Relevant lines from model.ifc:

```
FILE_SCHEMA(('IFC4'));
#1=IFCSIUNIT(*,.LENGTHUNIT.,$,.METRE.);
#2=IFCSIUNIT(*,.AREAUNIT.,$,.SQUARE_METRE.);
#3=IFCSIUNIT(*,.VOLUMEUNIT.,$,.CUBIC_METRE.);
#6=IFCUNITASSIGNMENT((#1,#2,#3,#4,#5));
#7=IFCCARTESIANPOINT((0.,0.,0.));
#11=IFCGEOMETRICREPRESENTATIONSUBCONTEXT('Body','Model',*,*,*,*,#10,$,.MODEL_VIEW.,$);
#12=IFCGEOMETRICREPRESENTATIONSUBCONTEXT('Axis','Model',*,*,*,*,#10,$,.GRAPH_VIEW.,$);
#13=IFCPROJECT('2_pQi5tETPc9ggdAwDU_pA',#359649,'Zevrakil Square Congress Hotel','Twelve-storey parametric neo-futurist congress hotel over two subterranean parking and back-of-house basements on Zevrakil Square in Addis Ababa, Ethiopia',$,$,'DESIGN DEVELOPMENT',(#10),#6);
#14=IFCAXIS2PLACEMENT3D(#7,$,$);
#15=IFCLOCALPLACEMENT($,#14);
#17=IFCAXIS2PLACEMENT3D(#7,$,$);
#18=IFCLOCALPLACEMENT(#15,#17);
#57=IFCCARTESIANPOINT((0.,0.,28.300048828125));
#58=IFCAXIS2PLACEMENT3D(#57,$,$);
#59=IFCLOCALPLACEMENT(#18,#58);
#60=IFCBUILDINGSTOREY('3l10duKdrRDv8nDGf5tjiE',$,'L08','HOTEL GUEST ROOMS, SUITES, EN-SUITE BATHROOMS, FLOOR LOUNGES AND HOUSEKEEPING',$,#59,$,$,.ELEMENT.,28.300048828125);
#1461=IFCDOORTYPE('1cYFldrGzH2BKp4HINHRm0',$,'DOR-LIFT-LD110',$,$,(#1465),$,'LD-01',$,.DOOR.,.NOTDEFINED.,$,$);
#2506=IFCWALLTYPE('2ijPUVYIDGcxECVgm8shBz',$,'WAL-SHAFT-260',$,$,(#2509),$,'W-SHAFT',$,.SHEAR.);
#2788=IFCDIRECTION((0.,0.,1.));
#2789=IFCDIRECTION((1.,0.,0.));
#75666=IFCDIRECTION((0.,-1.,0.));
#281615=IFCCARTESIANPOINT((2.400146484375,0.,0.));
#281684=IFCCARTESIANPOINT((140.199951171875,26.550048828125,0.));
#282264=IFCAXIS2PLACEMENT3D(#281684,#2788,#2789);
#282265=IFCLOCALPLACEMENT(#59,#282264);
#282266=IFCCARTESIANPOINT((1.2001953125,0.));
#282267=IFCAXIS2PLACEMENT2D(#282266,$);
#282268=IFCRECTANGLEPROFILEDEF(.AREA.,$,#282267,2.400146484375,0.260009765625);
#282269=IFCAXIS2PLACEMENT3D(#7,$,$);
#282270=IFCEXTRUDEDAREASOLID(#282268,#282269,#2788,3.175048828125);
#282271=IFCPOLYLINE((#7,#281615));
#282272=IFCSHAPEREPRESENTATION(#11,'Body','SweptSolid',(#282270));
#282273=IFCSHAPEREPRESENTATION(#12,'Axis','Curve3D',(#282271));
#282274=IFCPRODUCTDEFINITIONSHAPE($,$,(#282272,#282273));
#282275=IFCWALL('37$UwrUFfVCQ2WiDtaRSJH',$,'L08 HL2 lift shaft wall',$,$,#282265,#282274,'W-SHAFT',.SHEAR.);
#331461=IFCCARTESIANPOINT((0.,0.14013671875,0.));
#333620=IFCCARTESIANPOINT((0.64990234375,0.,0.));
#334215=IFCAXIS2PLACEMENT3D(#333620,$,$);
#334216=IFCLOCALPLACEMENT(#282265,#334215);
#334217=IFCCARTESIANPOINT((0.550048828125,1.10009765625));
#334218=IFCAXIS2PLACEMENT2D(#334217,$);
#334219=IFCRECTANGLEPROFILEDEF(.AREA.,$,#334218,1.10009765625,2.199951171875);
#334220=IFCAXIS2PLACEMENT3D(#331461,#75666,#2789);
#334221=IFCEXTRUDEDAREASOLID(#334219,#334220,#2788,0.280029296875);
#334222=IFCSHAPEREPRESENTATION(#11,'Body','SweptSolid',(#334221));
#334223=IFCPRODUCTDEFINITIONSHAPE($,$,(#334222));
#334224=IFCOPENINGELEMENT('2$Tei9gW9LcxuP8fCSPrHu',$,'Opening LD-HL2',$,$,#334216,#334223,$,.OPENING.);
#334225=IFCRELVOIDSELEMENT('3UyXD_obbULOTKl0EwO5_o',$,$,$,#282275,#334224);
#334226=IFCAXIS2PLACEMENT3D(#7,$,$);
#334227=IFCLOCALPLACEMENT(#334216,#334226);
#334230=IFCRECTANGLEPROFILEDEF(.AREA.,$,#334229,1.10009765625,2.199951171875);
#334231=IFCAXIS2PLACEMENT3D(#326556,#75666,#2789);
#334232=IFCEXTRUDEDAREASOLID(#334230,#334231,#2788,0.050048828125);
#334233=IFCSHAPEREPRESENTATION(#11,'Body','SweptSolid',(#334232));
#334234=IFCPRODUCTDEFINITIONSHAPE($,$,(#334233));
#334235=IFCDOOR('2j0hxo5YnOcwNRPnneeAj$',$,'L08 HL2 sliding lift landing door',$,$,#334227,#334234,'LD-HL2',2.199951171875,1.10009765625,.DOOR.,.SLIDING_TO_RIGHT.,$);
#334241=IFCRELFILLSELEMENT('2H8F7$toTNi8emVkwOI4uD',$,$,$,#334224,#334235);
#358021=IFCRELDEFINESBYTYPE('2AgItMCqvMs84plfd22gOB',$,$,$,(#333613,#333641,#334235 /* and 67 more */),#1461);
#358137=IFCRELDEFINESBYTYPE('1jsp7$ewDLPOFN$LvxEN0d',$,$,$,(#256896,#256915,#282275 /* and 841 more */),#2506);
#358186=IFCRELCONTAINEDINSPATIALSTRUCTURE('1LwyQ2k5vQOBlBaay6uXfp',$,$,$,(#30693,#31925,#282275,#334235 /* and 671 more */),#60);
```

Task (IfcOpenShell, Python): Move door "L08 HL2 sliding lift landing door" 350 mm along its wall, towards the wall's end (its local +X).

```python
import ifcopenshell
import ifcopenshell.api.geometry
import ifcopenshell.util.placement

model = ifcopenshell.open("model.ifc")

door = model.by_guid("2j0hxo5YnOcwNRPnneeAj$")
opening = door.FillsVoids[0].RelatingOpeningElement
wall = opening.VoidsElements[0].RelatingBuildingElement

wall_matrix = ifcopenshell.util.placement.get_local_placement(wall.ObjectPlacement)
shift = wall_matrix[:3, 0] * 0.35
before = ifcopenshell.util.placement.get_local_placement(door.ObjectPlacement)[:3, 3].copy()

# The door is placed relative to its opening, so it follows when the opening moves.
matrix = ifcopenshell.util.placement.get_local_placement(opening.ObjectPlacement)
matrix[:3, 3] += shift
ifcopenshell.api.geometry.edit_object_placement(
    model, product=opening, matrix=matrix, is_si=False, should_transform_children=True
)

after = ifcopenshell.util.placement.get_local_placement(door.ObjectPlacement)[:3, 3]
print("door moved by", (after - before).round(3) + 0.0)

model.write("model_rev.ifc")
```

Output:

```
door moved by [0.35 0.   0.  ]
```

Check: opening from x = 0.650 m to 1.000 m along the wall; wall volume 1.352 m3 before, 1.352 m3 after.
